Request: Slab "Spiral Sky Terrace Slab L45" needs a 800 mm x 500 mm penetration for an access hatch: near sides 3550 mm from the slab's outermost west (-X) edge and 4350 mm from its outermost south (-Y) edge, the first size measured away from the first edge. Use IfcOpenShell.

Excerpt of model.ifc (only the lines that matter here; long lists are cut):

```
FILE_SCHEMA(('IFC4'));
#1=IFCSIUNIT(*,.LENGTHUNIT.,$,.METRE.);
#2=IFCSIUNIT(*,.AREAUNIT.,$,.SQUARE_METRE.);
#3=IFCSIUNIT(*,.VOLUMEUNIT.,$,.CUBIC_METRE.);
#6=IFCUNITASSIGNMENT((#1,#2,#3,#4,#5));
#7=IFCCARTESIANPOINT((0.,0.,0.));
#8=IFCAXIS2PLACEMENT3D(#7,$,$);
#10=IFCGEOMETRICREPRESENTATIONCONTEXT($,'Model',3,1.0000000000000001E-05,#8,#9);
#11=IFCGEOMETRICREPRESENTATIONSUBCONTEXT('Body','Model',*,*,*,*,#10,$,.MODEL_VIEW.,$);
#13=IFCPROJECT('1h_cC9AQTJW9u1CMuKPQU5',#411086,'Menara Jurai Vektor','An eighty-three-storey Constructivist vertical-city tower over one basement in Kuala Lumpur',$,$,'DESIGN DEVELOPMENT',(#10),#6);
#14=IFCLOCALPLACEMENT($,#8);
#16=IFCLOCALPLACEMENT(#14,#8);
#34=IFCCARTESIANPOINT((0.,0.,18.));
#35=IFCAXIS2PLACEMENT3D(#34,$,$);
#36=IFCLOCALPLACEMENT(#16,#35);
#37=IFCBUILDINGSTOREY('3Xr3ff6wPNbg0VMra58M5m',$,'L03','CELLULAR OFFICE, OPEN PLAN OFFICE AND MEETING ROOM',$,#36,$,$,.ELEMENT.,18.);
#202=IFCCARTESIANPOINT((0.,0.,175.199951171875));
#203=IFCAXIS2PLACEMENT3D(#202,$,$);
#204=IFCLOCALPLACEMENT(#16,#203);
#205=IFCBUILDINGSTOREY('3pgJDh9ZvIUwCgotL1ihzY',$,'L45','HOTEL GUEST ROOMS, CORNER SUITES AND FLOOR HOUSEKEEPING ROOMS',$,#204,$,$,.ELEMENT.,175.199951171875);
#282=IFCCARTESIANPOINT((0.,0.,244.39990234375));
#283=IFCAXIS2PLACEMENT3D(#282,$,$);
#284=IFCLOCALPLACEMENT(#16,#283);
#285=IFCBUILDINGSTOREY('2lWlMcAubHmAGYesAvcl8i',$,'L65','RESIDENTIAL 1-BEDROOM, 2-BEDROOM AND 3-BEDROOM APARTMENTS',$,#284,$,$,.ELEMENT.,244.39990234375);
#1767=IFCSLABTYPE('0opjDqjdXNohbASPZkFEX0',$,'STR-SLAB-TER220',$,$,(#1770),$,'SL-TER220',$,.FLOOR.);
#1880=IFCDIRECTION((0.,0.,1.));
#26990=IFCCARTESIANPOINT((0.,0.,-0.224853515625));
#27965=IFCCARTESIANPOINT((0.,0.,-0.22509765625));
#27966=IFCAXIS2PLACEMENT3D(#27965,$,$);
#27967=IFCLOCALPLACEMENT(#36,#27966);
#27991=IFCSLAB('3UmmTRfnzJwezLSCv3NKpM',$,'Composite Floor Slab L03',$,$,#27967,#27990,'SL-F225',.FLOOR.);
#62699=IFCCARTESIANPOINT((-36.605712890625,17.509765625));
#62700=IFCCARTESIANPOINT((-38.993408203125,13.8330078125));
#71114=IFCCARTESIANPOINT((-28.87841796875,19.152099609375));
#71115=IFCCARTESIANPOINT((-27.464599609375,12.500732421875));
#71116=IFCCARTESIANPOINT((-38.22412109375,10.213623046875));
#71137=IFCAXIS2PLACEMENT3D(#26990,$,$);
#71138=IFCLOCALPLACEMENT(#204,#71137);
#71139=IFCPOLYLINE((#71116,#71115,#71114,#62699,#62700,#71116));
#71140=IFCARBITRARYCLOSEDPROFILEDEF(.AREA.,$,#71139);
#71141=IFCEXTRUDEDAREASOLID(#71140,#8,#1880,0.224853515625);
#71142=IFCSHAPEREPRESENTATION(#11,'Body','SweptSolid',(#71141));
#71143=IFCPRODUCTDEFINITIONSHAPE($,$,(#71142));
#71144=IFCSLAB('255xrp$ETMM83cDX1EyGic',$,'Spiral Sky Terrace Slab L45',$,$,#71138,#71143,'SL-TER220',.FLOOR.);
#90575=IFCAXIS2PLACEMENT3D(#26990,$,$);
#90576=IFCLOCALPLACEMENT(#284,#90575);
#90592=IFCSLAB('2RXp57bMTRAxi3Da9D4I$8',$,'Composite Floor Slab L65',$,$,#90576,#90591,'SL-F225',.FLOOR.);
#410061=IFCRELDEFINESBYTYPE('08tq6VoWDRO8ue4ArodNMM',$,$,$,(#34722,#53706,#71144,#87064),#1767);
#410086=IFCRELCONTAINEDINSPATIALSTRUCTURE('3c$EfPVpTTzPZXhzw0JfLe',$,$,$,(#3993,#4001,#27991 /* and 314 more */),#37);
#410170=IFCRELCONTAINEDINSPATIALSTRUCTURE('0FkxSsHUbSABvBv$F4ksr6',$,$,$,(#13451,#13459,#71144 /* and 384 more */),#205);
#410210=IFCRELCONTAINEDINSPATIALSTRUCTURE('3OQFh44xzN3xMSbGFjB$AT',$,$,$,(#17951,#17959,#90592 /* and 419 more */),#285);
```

```python
import numpy as np
import ifcopenshell
import ifcopenshell.api.feature
import ifcopenshell.api.geometry
import ifcopenshell.api.root
import ifcopenshell.geom
import ifcopenshell.util.placement
import ifcopenshell.util.representation
import ifcopenshell.util.shape
import ifcopenshell.util.unit

model = ifcopenshell.open("model.ifc")
unit_scale = ifcopenshell.util.unit.calculate_unit_scale(model)
settings = ifcopenshell.geom.settings()


def volume(element):
    """Net volume in cubic metres, openings subtracted."""
    shape = ifcopenshell.geom.create_shape(settings, element)
    return ifcopenshell.util.shape.get_volume(shape.geometry)


slab = model.by_guid("255xrp$ETMM83cDX1EyGic")
before = volume(slab)

# Extent in the slab's own axes, in metres. The edges named are its -X and -Y sides.
slab_shape = ifcopenshell.geom.create_shape(settings, slab)
vertices = ifcopenshell.util.shape.get_vertices(slab_shape.geometry)
x_min, y_min, bottom = vertices.min(axis=0)
top = vertices[:, 2].max()

opening = ifcopenshell.api.root.create_entity(model, ifc_class="IfcOpeningElement", name="Access hatch opening", predefined_type="OPENING")
context = ifcopenshell.util.representation.get_context(model, "Model", "Body", "MODEL_VIEW")
width, depth = 0.8, 0.5
outline = [(0.0, 0.0), (width, 0.0), (width, depth), (0.0, depth), (0.0, 0.0)]
# Overshoot both faces by 50 mm so the cut is clean.
shape = ifcopenshell.api.geometry.add_slab_representation(
    model, context=context, depth=top - bottom + 0.1, polyline=outline
)
ifcopenshell.api.geometry.assign_representation(model, product=opening, representation=shape)

matrix = ifcopenshell.util.placement.get_local_placement(slab.ObjectPlacement)
matrix[:, 3] = matrix @ np.append(np.array([x_min + 3.55, y_min + 4.35, bottom - 0.05]) / unit_scale, 1.0)
ifcopenshell.api.geometry.edit_object_placement(model, product=opening, matrix=matrix, is_si=False)
ifcopenshell.api.feature.add_feature(model, feature=opening, element=slab)

after = volume(slab)

print(f"slab volume {before:.3f} -> {after:.3f} m3")

model.write("model_updated.ifc")
```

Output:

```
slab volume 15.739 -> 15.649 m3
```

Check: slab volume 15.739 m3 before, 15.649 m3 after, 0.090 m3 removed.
